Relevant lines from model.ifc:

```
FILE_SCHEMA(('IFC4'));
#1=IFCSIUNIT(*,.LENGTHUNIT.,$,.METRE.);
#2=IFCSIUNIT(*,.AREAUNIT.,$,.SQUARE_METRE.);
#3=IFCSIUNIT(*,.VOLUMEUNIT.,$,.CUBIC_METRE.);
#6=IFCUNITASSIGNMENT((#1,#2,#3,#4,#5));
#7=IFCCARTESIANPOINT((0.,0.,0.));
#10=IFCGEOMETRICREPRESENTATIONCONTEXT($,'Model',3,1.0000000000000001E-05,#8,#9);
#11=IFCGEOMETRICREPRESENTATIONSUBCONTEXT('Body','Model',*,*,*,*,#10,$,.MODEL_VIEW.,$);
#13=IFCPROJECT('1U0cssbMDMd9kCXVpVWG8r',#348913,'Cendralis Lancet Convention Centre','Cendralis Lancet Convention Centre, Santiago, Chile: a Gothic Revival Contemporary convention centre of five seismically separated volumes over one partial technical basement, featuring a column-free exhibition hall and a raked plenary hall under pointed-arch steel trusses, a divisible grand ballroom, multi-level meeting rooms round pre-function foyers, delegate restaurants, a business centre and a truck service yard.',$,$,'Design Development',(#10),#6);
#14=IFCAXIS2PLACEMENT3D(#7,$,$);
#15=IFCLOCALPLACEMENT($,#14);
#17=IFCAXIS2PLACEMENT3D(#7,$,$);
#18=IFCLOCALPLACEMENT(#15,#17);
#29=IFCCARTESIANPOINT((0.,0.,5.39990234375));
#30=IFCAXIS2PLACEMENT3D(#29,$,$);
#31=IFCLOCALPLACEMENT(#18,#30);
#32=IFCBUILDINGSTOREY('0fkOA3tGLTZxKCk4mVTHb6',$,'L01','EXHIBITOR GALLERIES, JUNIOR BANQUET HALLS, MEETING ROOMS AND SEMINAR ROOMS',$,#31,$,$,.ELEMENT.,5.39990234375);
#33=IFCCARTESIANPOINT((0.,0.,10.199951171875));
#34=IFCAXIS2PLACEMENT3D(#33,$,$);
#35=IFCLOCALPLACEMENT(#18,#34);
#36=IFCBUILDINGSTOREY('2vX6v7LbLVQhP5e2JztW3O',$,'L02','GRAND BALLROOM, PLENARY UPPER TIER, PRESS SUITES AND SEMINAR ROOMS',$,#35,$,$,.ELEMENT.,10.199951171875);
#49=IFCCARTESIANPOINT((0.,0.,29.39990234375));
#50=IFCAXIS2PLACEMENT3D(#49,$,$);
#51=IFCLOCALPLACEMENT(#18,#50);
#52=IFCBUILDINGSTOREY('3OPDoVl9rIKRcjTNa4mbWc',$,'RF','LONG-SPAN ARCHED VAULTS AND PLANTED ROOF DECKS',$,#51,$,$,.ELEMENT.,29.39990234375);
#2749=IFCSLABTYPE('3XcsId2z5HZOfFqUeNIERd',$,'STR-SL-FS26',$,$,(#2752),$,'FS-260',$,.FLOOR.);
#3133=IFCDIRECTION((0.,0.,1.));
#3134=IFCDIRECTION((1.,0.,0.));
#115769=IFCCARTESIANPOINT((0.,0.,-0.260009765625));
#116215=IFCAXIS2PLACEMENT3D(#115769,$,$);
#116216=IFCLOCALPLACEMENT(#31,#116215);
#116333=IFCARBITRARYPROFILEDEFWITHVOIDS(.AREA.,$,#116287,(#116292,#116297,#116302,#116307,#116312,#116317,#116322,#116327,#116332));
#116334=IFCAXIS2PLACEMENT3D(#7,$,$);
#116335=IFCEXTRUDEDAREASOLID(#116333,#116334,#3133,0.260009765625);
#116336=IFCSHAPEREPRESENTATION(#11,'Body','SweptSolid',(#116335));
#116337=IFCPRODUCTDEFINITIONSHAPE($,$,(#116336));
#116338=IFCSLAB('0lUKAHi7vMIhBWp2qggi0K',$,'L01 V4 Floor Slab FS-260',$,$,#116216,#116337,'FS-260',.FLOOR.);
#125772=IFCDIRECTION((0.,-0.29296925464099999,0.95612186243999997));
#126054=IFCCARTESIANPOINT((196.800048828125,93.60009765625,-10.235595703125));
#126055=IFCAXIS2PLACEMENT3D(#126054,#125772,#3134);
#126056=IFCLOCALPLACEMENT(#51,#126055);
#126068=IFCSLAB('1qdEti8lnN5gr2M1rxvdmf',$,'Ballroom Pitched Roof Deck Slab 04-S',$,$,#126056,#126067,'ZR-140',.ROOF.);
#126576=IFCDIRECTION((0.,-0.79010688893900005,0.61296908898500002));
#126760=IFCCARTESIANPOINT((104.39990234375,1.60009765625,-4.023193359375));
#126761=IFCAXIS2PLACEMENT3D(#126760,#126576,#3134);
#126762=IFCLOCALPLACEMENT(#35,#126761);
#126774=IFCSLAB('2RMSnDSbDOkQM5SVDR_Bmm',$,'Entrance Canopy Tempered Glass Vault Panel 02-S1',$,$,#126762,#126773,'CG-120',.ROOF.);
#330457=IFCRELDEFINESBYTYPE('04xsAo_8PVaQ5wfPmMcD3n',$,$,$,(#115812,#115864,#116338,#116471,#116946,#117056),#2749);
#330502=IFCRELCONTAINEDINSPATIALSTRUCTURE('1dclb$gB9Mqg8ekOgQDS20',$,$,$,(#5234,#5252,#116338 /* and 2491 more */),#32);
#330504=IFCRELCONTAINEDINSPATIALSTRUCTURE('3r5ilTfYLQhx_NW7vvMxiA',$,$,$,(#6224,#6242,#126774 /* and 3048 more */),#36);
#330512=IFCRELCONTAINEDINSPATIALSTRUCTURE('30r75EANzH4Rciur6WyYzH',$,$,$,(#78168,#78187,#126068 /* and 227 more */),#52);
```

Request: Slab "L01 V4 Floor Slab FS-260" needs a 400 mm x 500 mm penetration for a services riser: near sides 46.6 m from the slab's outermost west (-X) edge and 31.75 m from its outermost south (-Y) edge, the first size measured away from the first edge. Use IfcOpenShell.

```python
import numpy as np
import ifcopenshell
import ifcopenshell.api.feature
import ifcopenshell.api.geometry
import ifcopenshell.api.root
import ifcopenshell.geom
import ifcopenshell.util.placement
import ifcopenshell.util.representation
import ifcopenshell.util.shape
import ifcopenshell.util.unit

model = ifcopenshell.open("model.ifc")
unit_scale = ifcopenshell.util.unit.calculate_unit_scale(model)
settings = ifcopenshell.geom.settings()


def volume(element):
    """Net volume in cubic metres, openings subtracted."""
    shape = ifcopenshell.geom.create_shape(settings, element)
    return ifcopenshell.util.shape.get_volume(shape.geometry)


slab = model.by_guid("0lUKAHi7vMIhBWp2qggi0K")
before = volume(slab)

# Extent in the slab's own axes, in metres. The edges named are its -X and -Y sides.
slab_shape = ifcopenshell.geom.create_shape(settings, slab)
vertices = ifcopenshell.util.shape.get_vertices(slab_shape.geometry)
x_min, y_min, bottom = vertices.min(axis=0)
top = vertices[:, 2].max()

opening = ifcopenshell.api.root.create_entity(model, ifc_class="IfcOpeningElement", name="Services riser opening", predefined_type="OPENING")
context = ifcopenshell.util.representation.get_context(model, "Model", "Body", "MODEL_VIEW")
width, depth = 0.4, 0.5
outline = [(0.0, 0.0), (width, 0.0), (width, depth), (0.0, depth), (0.0, 0.0)]
# Overshoot both faces by 50 mm so the cut is clean.
shape = ifcopenshell.api.geometry.add_slab_representation(
    model, context=context, depth=top - bottom + 0.1, polyline=outline
)
ifcopenshell.api.geometry.assign_representation(model, product=opening, representation=shape)

matrix = ifcopenshell.util.placement.get_local_placement(slab.ObjectPlacement)
matrix[:, 3] = matrix @ np.append(np.array([x_min + 46.6, y_min + 31.75, bottom - 0.05]) / unit_scale, 1.0)
ifcopenshell.api.geometry.edit_object_placement(model, product=opening, matrix=matrix, is_si=False)
ifcopenshell.api.feature.add_feature(model, feature=opening, element=slab)

after = volume(slab)

print(f"slab volume {before:.3f} -> {after:.3f} m3")

model.write("model_updated.ifc")
```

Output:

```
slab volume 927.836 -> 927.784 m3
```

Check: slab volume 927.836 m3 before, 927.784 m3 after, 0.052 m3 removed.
